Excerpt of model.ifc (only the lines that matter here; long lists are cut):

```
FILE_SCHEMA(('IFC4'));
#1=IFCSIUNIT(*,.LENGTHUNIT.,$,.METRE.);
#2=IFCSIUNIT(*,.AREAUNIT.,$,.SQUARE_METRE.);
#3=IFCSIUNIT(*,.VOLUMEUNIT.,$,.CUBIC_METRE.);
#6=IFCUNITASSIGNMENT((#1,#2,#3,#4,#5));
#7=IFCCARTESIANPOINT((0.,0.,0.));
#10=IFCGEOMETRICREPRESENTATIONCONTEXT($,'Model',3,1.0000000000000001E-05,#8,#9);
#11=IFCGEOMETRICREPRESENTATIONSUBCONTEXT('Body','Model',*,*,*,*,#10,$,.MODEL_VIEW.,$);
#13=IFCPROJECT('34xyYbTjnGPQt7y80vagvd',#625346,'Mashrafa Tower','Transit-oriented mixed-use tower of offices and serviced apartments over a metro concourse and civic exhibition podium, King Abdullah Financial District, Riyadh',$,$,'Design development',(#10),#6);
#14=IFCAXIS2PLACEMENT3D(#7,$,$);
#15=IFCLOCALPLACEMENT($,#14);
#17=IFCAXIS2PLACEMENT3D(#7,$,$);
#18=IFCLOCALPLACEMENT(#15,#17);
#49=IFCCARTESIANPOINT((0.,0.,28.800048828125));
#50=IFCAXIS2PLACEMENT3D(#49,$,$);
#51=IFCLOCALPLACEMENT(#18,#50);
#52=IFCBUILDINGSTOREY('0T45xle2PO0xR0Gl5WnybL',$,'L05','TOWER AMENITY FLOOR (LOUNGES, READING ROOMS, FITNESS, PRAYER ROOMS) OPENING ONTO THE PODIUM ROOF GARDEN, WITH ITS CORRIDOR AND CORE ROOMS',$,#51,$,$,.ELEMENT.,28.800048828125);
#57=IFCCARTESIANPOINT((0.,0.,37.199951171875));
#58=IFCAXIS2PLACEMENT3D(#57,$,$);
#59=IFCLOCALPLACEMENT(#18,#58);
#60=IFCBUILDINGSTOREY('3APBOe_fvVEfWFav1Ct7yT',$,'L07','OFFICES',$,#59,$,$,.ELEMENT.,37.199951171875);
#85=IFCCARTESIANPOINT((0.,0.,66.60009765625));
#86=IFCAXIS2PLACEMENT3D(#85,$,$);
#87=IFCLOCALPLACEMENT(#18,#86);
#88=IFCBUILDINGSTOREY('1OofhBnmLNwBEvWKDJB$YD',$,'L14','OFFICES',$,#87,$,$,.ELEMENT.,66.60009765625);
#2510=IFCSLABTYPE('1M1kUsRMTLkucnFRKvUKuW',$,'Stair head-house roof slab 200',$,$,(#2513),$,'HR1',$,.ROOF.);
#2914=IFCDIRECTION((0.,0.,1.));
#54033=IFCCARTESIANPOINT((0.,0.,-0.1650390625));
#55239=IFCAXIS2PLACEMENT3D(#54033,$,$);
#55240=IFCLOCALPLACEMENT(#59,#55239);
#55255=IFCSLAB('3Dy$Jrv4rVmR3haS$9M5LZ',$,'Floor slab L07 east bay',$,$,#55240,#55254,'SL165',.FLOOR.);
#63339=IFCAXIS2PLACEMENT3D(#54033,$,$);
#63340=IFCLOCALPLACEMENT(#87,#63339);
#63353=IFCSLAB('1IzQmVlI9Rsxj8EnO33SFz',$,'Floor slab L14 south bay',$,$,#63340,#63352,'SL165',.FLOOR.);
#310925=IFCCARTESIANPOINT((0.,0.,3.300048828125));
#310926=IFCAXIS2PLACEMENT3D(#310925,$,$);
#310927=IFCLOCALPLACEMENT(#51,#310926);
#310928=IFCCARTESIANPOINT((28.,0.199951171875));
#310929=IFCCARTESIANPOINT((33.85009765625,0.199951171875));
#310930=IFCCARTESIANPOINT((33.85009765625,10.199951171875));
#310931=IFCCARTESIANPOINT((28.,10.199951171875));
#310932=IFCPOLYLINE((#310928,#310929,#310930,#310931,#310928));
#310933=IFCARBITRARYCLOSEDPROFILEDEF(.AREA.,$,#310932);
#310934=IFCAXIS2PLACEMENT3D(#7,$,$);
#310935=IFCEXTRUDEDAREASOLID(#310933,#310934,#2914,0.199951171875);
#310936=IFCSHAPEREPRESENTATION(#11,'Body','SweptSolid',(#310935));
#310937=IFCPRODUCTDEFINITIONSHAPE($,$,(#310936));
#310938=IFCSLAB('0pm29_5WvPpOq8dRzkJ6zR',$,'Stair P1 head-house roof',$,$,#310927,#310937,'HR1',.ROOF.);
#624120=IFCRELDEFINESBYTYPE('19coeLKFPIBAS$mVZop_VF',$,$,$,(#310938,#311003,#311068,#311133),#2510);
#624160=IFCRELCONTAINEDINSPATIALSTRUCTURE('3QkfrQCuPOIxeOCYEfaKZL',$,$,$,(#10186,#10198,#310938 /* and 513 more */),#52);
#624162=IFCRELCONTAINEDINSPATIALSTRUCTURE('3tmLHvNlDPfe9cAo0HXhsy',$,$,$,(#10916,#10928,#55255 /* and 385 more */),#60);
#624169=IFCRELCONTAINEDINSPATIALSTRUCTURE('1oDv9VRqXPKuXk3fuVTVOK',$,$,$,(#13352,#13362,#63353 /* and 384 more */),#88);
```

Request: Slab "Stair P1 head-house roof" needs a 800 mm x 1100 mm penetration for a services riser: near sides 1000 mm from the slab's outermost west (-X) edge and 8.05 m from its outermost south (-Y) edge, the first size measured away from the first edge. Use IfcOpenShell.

```python
import numpy as np
import ifcopenshell
import ifcopenshell.api.feature
import ifcopenshell.api.geometry
import ifcopenshell.api.root
import ifcopenshell.geom
import ifcopenshell.util.placement
import ifcopenshell.util.representation
import ifcopenshell.util.shape
import ifcopenshell.util.unit

model = ifcopenshell.open("model.ifc")
unit_scale = ifcopenshell.util.unit.calculate_unit_scale(model)
settings = ifcopenshell.geom.settings()


def volume(element):
    """Net volume in cubic metres, openings subtracted."""
    shape = ifcopenshell.geom.create_shape(settings, element)
    return ifcopenshell.util.shape.get_volume(shape.geometry)


slab = model.by_guid("0pm29_5WvPpOq8dRzkJ6zR")
before = volume(slab)

# Extent in the slab's own axes, in metres. The edges named are its -X and -Y sides.
slab_shape = ifcopenshell.geom.create_shape(settings, slab)
vertices = ifcopenshell.util.shape.get_vertices(slab_shape.geometry)
x_min, y_min, bottom = vertices.min(axis=0)
top = vertices[:, 2].max()

opening = ifcopenshell.api.root.create_entity(model, ifc_class="IfcOpeningElement", name="Services riser opening", predefined_type="OPENING")
context = ifcopenshell.util.representation.get_context(model, "Model", "Body", "MODEL_VIEW")
width, depth = 0.8, 1.1
outline = [(0.0, 0.0), (width, 0.0), (width, depth), (0.0, depth), (0.0, 0.0)]
# Overshoot both faces by 50 mm so the cut is clean.
shape = ifcopenshell.api.geometry.add_slab_representation(
    model, context=context, depth=top - bottom + 0.1, polyline=outline
)
ifcopenshell.api.geometry.assign_representation(model, product=opening, representation=shape)

matrix = ifcopenshell.util.placement.get_local_placement(slab.ObjectPlacement)
matrix[:, 3] = matrix @ np.append(np.array([x_min + 1, y_min + 8.05, bottom - 0.05]) / unit_scale, 1.0)
ifcopenshell.api.geometry.edit_object_placement(model, product=opening, matrix=matrix, is_si=False)
ifcopenshell.api.feature.add_feature(model, feature=opening, element=slab)

after = volume(slab)

print(f"slab volume {before:.3f} -> {after:.3f} m3")

model.write("model_rev.ifc")
```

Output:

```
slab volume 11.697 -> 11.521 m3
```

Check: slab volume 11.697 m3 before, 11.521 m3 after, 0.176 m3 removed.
